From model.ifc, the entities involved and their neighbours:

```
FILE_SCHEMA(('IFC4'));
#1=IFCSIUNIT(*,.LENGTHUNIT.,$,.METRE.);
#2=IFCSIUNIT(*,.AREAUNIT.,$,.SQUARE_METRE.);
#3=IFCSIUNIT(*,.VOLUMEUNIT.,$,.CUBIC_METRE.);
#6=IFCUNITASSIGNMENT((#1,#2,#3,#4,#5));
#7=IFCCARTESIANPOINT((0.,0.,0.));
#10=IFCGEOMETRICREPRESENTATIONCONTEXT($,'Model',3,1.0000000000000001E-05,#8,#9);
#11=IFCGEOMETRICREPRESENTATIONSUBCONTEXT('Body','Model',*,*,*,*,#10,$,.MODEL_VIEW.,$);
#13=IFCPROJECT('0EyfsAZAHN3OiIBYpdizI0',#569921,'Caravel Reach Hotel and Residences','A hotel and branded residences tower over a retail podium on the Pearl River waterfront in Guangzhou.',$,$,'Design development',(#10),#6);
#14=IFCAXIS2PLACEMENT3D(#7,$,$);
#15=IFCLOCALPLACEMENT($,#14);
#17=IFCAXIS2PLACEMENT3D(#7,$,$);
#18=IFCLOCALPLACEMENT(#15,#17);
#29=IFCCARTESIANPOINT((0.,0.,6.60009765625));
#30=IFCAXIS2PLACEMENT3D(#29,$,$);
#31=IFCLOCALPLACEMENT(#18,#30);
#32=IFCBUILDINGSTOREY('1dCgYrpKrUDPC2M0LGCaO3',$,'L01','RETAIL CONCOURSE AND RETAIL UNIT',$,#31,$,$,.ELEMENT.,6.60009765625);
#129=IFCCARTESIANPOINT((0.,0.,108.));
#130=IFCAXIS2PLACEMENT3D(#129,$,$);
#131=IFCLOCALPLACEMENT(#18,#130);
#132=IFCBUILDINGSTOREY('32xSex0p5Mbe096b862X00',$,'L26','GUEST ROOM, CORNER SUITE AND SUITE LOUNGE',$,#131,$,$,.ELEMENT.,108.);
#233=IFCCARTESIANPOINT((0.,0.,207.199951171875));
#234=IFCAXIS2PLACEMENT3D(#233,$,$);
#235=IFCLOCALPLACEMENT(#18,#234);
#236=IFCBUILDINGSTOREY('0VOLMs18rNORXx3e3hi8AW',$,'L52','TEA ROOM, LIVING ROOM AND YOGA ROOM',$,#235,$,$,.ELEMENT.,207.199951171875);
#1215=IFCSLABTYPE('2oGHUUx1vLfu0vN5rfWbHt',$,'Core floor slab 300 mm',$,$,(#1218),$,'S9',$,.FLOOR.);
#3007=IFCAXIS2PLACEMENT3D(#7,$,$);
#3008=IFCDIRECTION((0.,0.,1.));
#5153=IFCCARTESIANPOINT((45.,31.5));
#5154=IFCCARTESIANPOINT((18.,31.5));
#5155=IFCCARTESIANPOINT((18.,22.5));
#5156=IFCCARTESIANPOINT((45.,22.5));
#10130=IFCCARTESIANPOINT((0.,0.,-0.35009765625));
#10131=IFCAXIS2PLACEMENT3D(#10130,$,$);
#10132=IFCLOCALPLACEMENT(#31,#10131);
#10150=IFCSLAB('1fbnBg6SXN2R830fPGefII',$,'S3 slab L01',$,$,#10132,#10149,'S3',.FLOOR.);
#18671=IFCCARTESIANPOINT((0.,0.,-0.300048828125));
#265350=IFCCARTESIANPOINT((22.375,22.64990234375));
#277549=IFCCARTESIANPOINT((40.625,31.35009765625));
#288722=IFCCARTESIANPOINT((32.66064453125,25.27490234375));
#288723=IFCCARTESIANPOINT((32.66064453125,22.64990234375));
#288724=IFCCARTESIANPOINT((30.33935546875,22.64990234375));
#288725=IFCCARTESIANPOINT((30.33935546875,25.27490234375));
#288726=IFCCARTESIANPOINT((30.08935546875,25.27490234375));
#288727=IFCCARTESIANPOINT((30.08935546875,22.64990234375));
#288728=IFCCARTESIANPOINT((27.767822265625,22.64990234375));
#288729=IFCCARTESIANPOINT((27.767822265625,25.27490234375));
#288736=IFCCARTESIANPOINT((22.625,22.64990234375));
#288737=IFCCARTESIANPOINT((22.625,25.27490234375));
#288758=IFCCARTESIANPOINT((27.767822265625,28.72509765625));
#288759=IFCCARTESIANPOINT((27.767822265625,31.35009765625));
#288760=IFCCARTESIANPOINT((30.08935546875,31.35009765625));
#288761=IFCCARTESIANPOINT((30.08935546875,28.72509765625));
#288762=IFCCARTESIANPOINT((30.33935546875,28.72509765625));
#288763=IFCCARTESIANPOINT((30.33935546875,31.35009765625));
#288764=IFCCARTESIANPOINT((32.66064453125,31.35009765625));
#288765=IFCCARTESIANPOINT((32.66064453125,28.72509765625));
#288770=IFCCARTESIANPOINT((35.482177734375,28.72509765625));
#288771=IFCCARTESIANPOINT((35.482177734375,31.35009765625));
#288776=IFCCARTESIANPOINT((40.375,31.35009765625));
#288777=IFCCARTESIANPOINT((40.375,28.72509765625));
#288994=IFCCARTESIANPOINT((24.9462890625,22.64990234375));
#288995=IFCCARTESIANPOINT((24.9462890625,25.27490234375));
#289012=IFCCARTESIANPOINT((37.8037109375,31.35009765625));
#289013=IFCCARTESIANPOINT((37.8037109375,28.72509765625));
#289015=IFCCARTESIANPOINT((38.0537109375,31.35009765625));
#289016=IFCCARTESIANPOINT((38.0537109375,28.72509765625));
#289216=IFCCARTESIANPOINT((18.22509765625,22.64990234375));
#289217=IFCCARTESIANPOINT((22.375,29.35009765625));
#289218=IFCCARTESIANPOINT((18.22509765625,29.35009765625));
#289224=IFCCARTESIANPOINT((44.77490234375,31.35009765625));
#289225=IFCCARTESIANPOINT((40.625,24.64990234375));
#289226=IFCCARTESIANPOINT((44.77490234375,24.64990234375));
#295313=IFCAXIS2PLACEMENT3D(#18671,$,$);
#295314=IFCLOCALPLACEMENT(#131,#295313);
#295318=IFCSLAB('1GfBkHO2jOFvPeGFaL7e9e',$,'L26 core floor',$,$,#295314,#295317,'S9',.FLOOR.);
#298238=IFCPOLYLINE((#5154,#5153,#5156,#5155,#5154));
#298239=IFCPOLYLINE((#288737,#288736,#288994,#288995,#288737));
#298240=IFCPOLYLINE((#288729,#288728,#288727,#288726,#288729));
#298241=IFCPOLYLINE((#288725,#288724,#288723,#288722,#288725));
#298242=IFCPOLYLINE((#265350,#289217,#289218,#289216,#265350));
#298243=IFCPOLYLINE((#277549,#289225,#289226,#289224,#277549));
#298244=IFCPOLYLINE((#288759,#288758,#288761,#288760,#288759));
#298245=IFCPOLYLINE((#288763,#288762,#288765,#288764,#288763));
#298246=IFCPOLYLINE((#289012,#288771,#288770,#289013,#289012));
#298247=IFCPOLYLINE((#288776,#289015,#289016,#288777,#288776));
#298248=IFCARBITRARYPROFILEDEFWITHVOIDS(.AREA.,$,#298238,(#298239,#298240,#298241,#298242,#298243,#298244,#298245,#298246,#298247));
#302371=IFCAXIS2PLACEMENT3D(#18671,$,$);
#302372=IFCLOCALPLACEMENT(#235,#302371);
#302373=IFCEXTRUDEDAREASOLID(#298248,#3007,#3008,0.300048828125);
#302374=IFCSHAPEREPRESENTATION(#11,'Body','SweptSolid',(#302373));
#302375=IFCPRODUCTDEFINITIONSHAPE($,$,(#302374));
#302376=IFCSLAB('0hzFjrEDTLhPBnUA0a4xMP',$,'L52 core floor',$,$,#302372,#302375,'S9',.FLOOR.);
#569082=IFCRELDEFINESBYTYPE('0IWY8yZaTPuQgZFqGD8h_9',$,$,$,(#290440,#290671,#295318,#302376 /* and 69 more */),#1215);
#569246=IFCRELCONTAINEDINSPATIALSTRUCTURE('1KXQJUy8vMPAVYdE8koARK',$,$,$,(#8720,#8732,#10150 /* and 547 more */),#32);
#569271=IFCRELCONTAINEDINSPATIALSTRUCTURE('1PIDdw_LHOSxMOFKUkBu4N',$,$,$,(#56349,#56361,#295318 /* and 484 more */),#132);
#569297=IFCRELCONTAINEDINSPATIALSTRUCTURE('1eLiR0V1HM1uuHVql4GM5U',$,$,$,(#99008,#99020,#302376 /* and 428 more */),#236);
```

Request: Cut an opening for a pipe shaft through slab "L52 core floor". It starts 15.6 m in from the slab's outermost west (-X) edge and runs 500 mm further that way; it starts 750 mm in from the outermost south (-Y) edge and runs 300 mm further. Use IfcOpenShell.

```python
import numpy as np
import ifcopenshell
import ifcopenshell.api.feature
import ifcopenshell.api.geometry
import ifcopenshell.api.root
import ifcopenshell.geom
import ifcopenshell.util.placement
import ifcopenshell.util.representation
import ifcopenshell.util.shape
import ifcopenshell.util.unit

model = ifcopenshell.open("model.ifc")
unit_scale = ifcopenshell.util.unit.calculate_unit_scale(model)
settings = ifcopenshell.geom.settings()


def volume(element):
    """Net volume in cubic metres, openings subtracted."""
    shape = ifcopenshell.geom.create_shape(settings, element)
    return ifcopenshell.util.shape.get_volume(shape.geometry)


slab = model.by_id(302376)
before = volume(slab)

# Extent in the slab's own axes, in metres. The edges named are its -X and -Y sides.
slab_shape = ifcopenshell.geom.create_shape(settings, slab)
vertices = ifcopenshell.util.shape.get_vertices(slab_shape.geometry)
x_min, y_min, bottom = vertices.min(axis=0)
top = vertices[:, 2].max()

opening = ifcopenshell.api.root.create_entity(model, ifc_class="IfcOpeningElement", name="Pipe shaft opening", predefined_type="OPENING")
context = ifcopenshell.util.representation.get_context(model, "Model", "Body", "MODEL_VIEW")
width, depth = 0.5, 0.3
outline = [(0.0, 0.0), (width, 0.0), (width, depth), (0.0, depth), (0.0, 0.0)]
# Overshoot both faces by 50 mm so the cut is clean.
shape = ifcopenshell.api.geometry.add_slab_representation(
    model, context=context, depth=top - bottom + 0.1, polyline=outline
)
ifcopenshell.api.geometry.assign_representation(model, product=opening, representation=shape)

matrix = ifcopenshell.util.placement.get_local_placement(slab.ObjectPlacement)
matrix[:, 3] = matrix @ np.append(np.array([x_min + 15.6, y_min + 0.75, bottom - 0.05]) / unit_scale, 1.0)
ifcopenshell.api.geometry.edit_object_placement(model, product=opening, matrix=matrix, is_si=False)
ifcopenshell.api.feature.add_feature(model, feature=opening, element=slab)

after = volume(slab)

print(f"slab volume {before:.3f} -> {after:.3f} m3")

model.write("model_v2.ifc")
```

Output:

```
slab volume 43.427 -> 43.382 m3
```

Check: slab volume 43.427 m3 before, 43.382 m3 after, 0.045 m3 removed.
